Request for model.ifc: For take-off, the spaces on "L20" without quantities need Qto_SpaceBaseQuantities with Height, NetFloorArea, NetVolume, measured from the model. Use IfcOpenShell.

First a look at what the model holds.

```python
import ifcopenshell
import ifcopenshell.util.element
import ifcopenshell.util.unit

model = ifcopenshell.open("model.ifc")
print(model.schema)
for unit_type in ("LENGTHUNIT", "AREAUNIT", "VOLUMEUNIT"):
    print(unit_type, ifcopenshell.util.unit.calculate_unit_scale(model, unit_type))
storey = next(s for s in model.by_type("IfcBuildingStorey") if s.Name == "L20")
spaces = [e for e in ifcopenshell.util.element.get_decomposition(storey) if e.is_a("IfcSpace")]
for e in sorted(spaces, key=lambda e: e.id()):
    print(e.id(), e.is_a(), e.Name, list(ifcopenshell.util.element.get_psets(e, qtos_only=True)), sep=" | ")
```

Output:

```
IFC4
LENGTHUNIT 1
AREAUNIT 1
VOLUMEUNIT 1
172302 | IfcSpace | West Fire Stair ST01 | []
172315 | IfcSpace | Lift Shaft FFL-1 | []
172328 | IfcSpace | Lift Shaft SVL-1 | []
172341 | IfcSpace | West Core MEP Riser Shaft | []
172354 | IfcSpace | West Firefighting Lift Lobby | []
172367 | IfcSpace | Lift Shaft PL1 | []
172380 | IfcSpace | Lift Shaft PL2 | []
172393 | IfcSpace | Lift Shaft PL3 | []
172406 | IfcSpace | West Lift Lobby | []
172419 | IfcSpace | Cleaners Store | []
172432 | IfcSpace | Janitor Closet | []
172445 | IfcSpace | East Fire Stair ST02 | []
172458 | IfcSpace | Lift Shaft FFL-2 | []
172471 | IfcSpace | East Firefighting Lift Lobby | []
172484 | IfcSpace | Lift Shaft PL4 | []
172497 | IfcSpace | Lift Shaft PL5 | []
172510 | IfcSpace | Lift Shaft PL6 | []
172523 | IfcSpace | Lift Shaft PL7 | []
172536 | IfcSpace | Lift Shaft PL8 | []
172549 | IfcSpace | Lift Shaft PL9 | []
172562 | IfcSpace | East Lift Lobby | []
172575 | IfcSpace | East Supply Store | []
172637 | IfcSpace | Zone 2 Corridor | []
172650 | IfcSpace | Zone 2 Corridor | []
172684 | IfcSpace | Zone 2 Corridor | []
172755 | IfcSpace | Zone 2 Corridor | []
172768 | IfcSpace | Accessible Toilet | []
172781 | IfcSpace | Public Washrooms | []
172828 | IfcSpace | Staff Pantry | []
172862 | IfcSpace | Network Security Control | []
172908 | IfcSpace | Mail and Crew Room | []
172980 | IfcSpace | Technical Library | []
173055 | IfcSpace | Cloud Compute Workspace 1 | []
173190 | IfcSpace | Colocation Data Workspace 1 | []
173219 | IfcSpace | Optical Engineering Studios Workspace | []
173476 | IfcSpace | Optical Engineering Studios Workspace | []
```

```python
import ifcopenshell
import ifcopenshell.api.pset
import ifcopenshell.geom
import ifcopenshell.util.element
import ifcopenshell.util.shape
import ifcopenshell.util.unit

model = ifcopenshell.open("model.ifc")
unit_scale = ifcopenshell.util.unit.calculate_unit_scale(model)
area_scale = ifcopenshell.util.unit.calculate_unit_scale(model, "AREAUNIT")
volume_scale = ifcopenshell.util.unit.calculate_unit_scale(model, "VOLUMEUNIT")
settings = ifcopenshell.geom.settings()

storey = next(s for s in model.by_type("IfcBuildingStorey") if s.Name == "L20")
spaces = [e for e in ifcopenshell.util.element.get_decomposition(storey) if e.is_a("IfcSpace")]

for e in sorted(spaces, key=lambda e: e.id()):
    if ifcopenshell.util.element.get_psets(e, qtos_only=True, should_inherit=False):
        continue
    # Geometry comes back in metres, in the element's own axes.
    shape = ifcopenshell.geom.create_shape(settings, e)
    values = {
        "Height": ifcopenshell.util.shape.get_z(shape.geometry) / unit_scale,
        "NetFloorArea": ifcopenshell.util.shape.get_footprint_area(shape.geometry) / area_scale,
        "NetVolume": ifcopenshell.util.shape.get_volume(shape.geometry) / volume_scale,
    }
    qto = ifcopenshell.api.pset.add_qto(model, product=e, name="Qto_SpaceBaseQuantities")
    ifcopenshell.api.pset.edit_qto(model, qto=qto, properties=values)
    print(e.id(), {k: round(v, 3) for k, v in values.items()})

model.write("model_v2.ifc")
```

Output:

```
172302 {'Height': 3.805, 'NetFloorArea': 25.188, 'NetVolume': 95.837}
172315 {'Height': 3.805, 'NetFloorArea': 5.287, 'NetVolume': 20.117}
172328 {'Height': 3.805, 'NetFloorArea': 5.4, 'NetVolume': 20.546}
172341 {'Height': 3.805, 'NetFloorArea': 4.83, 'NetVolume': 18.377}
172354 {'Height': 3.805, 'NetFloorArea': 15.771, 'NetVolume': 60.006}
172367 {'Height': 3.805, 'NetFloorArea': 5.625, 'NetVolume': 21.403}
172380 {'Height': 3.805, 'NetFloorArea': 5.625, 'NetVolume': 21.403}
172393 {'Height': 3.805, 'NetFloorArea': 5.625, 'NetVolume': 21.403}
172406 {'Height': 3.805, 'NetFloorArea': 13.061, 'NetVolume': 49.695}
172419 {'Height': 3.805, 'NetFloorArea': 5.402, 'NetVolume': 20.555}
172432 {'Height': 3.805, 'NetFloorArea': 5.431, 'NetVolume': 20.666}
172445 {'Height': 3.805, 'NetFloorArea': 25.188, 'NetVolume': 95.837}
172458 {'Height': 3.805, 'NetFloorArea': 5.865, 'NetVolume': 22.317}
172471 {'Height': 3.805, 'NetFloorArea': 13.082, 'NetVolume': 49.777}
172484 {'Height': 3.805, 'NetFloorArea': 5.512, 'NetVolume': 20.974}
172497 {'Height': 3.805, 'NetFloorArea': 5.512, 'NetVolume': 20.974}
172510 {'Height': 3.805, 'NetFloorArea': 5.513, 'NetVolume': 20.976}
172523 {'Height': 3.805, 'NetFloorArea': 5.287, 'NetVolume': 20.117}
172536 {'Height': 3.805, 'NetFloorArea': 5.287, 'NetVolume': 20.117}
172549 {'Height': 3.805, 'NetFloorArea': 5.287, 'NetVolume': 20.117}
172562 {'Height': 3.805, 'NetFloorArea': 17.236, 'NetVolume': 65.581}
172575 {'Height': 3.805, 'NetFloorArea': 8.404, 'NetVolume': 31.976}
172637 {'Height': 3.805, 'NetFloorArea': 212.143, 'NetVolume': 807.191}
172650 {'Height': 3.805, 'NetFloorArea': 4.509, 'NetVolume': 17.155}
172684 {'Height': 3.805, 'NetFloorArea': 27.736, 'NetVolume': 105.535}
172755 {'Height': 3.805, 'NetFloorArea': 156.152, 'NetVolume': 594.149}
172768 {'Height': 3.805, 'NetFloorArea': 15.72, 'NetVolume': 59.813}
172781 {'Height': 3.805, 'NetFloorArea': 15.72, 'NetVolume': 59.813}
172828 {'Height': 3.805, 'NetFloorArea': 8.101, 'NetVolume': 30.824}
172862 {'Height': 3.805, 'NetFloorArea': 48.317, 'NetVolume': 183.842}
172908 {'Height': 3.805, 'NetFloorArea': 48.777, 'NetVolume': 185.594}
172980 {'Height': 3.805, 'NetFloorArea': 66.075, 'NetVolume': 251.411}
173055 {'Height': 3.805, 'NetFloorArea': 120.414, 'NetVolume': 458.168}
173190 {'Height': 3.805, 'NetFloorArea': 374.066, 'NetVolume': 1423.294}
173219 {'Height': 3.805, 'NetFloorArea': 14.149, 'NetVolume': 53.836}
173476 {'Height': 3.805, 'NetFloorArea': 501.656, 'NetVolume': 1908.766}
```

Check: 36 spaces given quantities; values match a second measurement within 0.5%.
